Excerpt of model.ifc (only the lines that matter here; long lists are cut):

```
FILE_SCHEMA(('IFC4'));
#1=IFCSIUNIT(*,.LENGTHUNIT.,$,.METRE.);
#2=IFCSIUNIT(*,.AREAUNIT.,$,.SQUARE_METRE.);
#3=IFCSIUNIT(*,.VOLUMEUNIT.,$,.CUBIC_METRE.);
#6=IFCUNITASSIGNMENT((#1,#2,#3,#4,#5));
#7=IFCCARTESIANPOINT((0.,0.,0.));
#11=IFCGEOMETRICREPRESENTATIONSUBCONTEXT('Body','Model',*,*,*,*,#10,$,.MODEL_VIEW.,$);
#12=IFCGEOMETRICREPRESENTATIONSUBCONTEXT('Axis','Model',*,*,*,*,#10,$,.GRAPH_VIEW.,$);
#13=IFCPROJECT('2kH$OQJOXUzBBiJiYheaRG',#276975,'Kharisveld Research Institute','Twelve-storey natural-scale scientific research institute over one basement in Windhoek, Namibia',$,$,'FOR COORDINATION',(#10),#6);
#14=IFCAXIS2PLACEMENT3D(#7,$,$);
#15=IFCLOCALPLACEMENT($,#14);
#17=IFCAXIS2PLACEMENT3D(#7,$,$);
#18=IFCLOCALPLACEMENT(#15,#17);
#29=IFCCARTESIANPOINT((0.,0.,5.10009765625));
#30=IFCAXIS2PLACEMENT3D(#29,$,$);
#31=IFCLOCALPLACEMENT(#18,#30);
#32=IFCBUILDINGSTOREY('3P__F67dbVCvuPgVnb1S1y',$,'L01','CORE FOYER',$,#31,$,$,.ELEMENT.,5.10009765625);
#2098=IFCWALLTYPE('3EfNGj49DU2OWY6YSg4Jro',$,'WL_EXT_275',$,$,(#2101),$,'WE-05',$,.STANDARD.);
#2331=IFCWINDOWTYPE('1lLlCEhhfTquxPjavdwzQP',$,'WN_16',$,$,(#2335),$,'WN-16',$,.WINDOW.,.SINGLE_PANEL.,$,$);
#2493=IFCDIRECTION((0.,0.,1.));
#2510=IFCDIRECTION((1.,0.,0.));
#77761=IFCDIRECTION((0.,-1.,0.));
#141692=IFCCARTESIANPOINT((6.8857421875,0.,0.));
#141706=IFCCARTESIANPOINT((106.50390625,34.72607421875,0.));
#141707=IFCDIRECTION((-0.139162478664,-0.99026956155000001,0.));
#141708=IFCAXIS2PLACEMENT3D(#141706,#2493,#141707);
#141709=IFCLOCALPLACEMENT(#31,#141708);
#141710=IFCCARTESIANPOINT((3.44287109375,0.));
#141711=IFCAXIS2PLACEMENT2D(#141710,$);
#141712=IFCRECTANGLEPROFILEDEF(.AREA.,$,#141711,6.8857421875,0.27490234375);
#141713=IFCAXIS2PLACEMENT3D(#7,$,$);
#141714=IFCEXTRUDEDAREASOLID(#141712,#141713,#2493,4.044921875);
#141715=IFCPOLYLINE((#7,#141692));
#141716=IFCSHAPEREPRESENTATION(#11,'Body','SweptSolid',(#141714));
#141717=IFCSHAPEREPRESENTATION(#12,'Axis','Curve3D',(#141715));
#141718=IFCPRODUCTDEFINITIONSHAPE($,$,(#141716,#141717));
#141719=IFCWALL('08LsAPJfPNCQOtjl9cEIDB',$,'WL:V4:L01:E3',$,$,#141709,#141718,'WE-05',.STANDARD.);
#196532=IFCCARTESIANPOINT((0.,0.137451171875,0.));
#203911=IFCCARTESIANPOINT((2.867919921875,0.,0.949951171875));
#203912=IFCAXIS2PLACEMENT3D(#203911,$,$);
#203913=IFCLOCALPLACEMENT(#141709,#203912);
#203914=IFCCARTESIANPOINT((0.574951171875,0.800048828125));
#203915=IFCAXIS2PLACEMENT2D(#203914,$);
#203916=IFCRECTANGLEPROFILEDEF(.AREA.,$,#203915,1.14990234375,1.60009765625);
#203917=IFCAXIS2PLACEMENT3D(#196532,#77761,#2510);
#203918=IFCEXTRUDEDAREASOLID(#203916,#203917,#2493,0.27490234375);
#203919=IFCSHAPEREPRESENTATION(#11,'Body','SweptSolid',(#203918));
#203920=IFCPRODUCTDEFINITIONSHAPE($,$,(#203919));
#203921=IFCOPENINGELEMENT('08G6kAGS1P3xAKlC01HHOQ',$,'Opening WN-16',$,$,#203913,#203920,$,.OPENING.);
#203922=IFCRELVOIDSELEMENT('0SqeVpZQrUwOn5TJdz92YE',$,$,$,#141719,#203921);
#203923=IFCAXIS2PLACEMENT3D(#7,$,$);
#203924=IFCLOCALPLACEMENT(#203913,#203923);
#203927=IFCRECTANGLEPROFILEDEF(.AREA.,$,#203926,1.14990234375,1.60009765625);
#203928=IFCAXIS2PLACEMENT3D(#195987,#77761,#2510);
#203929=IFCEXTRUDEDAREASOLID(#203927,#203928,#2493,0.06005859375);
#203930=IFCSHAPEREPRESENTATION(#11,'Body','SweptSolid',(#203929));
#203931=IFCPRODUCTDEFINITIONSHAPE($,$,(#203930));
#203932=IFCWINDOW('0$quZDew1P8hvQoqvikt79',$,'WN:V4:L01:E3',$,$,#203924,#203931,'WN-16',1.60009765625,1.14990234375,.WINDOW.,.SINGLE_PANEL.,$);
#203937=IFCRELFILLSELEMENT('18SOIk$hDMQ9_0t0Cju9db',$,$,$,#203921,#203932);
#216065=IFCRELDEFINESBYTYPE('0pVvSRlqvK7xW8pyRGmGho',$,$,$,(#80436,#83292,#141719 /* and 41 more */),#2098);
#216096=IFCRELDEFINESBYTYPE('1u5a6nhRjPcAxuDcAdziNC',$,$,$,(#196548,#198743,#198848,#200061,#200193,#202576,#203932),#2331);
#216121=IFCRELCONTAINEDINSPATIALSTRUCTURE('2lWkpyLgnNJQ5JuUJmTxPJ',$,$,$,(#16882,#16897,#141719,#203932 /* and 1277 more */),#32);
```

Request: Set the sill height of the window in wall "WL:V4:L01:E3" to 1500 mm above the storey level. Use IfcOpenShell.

```python
import numpy as np
import ifcopenshell
import ifcopenshell.api.geometry
import ifcopenshell.geom
import ifcopenshell.util.element
import ifcopenshell.util.placement
import ifcopenshell.util.shape
import ifcopenshell.util.unit

model = ifcopenshell.open("model.ifc")
unit_scale = ifcopenshell.util.unit.calculate_unit_scale(model)

window = model.by_guid("0$quZDew1P8hvQoqvikt79")
opening = window.FillsVoids[0].RelatingOpeningElement
storey = ifcopenshell.util.element.get_container(window, ifc_class="IfcBuildingStorey")
level = ifcopenshell.util.placement.get_local_placement(storey.ObjectPlacement)[2, 3]

# The opening's origin need not be at the sill, so measure its lowest point.
shape = ifcopenshell.geom.create_shape(ifcopenshell.geom.settings(), opening)
bottom = ifcopenshell.util.shape.get_shape_bottom_elevation(shape, shape.geometry) / unit_scale
dz = level + 1.5 - bottom

shift = np.array([0.0, 0.0, dz])
# The window is placed relative to its opening, so it follows when the opening moves.
matrix = ifcopenshell.util.placement.get_local_placement(opening.ObjectPlacement)
matrix[:3, 3] += shift
ifcopenshell.api.geometry.edit_object_placement(
    model, product=opening, matrix=matrix, is_si=False, should_transform_children=True
)

print(f"moved by {dz * unit_scale:+.3f} m")

model.write("model_v2.ifc")
```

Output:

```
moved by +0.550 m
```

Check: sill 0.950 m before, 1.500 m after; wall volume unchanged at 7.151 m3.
